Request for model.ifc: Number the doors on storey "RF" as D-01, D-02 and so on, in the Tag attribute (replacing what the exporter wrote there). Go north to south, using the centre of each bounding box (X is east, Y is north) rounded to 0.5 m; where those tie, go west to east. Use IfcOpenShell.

First a look at what the model holds.

```python
import ifcopenshell
import ifcopenshell.util.element
import ifcopenshell.util.placement

model = ifcopenshell.open("model.ifc")
print(model.schema)
storey = next(s for s in model.by_type("IfcBuildingStorey") if s.Name == "RF")
doors = [e for e in ifcopenshell.util.element.get_decomposition(storey) if e.is_a("IfcDoor")]
for e in sorted(doors, key=lambda e: e.id()):
    origin = ifcopenshell.util.placement.get_local_placement(e.ObjectPlacement)[:3, 3]
    print(e.id(), e.Tag, e.Name, origin.round(2) + 0.0, sep=" | ")
```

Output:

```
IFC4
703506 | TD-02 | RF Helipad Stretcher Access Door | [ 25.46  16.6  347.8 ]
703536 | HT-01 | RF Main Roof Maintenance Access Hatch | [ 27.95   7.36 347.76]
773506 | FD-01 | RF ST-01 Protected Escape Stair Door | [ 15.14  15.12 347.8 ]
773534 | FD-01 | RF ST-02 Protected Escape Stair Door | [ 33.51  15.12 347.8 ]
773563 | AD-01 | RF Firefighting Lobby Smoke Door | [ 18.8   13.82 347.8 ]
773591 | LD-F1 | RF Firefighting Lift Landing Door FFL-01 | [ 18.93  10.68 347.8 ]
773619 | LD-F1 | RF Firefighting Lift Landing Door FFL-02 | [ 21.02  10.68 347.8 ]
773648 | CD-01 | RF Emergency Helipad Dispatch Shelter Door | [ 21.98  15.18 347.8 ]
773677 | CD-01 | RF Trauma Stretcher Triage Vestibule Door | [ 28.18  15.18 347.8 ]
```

```python
import ifcopenshell
import ifcopenshell.geom
import ifcopenshell.util.element
import ifcopenshell.util.shape

model = ifcopenshell.open("model.ifc")
settings = ifcopenshell.geom.settings()
settings.set("use-world-coords", True)


def centre(element):
    shape = ifcopenshell.geom.create_shape(settings, element)
    return ifcopenshell.util.shape.get_bbox_centroid(shape.geometry)


storey = next(s for s in model.by_type("IfcBuildingStorey") if s.Name == "RF")
doors = [e for e in ifcopenshell.util.element.get_decomposition(storey) if e.is_a("IfcDoor")]

# Insertion points can sit at a corner or the storey origin, so sort by the geometry (in metres).
centres = {e: centre(e) for e in doors}
doors.sort(key=lambda e: (-round(centres[e][1] / 0.5), centres[e][0]))

for i, e in enumerate(doors, start=1):
    number = f"D-{i:02d}"
    e.Tag = number
    print(e.id(), number)

model.write("model_edited.ifc")
```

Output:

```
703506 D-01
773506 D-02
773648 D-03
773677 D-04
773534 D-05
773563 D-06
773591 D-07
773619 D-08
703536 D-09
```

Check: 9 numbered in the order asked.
